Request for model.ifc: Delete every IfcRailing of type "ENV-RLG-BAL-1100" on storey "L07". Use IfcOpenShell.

First a look at what the model holds.

```python
import ifcopenshell
import ifcopenshell.util.element

model = ifcopenshell.open("model.ifc")
print(model.schema)
storey = next(s for s in model.by_type("IfcBuildingStorey") if s.Name == "L07")
railings = [e for e in ifcopenshell.util.element.get_decomposition(storey) if e.is_a("IfcRailing")]
seen = {}
for e in railings:
    element_type = ifcopenshell.util.element.get_type(e)
    name = element_type.Name if element_type not in (None, e) else None
    seen[name] = seen.get(name, 0) + 1
for name, count in sorted(seen.items(), key=str):
    print(count, "x", name)
```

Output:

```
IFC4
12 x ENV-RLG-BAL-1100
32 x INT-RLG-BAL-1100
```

```python
import ifcopenshell
import ifcopenshell.api.root
import ifcopenshell.util.element

model = ifcopenshell.open("model.ifc")

storey = next(s for s in model.by_type("IfcBuildingStorey") if s.Name == "L07")
railings = [e for e in ifcopenshell.util.element.get_decomposition(storey) if e.is_a("IfcRailing")]
targets = [e for e in railings if (t := ifcopenshell.util.element.get_type(e)) not in (None, e) and t.Name == "ENV-RLG-BAL-1100"]

for e in targets:
    ifcopenshell.api.root.remove_product(model, product=e)
print(len(targets), "removed")

model.write("model_edited.ifc")
```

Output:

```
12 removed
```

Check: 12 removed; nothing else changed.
